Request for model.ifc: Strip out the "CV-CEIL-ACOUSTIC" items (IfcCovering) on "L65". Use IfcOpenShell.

First a look at what the model holds.

```python
import ifcopenshell
import ifcopenshell.util.element

model = ifcopenshell.open("model.ifc")
print(model.schema)
storey = next(s for s in model.by_type("IfcBuildingStorey") if s.Name == "L65")
coverings = [e for e in ifcopenshell.util.element.get_decomposition(storey) if e.is_a("IfcCovering")]
seen = {}
for e in coverings:
    element_type = ifcopenshell.util.element.get_type(e)
    name = element_type.Name if element_type not in (None, e) else None
    seen[name] = seen.get(name, 0) + 1
for name, count in sorted(seen.items(), key=str):
    print(count, "x", name)
```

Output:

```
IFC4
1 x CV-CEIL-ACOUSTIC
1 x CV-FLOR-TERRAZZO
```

```python
import ifcopenshell
import ifcopenshell.api.root
import ifcopenshell.util.element

model = ifcopenshell.open("model.ifc")

storey = next(s for s in model.by_type("IfcBuildingStorey") if s.Name == "L65")
coverings = [e for e in ifcopenshell.util.element.get_decomposition(storey) if e.is_a("IfcCovering")]
targets = [e for e in coverings if (t := ifcopenshell.util.element.get_type(e)) not in (None, e) and t.Name == "CV-CEIL-ACOUSTIC"]

for e in targets:
    ifcopenshell.api.root.remove_product(model, product=e)
print(len(targets), "removed")

model.write("model_edited.ifc")
```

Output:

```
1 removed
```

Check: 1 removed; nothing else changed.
